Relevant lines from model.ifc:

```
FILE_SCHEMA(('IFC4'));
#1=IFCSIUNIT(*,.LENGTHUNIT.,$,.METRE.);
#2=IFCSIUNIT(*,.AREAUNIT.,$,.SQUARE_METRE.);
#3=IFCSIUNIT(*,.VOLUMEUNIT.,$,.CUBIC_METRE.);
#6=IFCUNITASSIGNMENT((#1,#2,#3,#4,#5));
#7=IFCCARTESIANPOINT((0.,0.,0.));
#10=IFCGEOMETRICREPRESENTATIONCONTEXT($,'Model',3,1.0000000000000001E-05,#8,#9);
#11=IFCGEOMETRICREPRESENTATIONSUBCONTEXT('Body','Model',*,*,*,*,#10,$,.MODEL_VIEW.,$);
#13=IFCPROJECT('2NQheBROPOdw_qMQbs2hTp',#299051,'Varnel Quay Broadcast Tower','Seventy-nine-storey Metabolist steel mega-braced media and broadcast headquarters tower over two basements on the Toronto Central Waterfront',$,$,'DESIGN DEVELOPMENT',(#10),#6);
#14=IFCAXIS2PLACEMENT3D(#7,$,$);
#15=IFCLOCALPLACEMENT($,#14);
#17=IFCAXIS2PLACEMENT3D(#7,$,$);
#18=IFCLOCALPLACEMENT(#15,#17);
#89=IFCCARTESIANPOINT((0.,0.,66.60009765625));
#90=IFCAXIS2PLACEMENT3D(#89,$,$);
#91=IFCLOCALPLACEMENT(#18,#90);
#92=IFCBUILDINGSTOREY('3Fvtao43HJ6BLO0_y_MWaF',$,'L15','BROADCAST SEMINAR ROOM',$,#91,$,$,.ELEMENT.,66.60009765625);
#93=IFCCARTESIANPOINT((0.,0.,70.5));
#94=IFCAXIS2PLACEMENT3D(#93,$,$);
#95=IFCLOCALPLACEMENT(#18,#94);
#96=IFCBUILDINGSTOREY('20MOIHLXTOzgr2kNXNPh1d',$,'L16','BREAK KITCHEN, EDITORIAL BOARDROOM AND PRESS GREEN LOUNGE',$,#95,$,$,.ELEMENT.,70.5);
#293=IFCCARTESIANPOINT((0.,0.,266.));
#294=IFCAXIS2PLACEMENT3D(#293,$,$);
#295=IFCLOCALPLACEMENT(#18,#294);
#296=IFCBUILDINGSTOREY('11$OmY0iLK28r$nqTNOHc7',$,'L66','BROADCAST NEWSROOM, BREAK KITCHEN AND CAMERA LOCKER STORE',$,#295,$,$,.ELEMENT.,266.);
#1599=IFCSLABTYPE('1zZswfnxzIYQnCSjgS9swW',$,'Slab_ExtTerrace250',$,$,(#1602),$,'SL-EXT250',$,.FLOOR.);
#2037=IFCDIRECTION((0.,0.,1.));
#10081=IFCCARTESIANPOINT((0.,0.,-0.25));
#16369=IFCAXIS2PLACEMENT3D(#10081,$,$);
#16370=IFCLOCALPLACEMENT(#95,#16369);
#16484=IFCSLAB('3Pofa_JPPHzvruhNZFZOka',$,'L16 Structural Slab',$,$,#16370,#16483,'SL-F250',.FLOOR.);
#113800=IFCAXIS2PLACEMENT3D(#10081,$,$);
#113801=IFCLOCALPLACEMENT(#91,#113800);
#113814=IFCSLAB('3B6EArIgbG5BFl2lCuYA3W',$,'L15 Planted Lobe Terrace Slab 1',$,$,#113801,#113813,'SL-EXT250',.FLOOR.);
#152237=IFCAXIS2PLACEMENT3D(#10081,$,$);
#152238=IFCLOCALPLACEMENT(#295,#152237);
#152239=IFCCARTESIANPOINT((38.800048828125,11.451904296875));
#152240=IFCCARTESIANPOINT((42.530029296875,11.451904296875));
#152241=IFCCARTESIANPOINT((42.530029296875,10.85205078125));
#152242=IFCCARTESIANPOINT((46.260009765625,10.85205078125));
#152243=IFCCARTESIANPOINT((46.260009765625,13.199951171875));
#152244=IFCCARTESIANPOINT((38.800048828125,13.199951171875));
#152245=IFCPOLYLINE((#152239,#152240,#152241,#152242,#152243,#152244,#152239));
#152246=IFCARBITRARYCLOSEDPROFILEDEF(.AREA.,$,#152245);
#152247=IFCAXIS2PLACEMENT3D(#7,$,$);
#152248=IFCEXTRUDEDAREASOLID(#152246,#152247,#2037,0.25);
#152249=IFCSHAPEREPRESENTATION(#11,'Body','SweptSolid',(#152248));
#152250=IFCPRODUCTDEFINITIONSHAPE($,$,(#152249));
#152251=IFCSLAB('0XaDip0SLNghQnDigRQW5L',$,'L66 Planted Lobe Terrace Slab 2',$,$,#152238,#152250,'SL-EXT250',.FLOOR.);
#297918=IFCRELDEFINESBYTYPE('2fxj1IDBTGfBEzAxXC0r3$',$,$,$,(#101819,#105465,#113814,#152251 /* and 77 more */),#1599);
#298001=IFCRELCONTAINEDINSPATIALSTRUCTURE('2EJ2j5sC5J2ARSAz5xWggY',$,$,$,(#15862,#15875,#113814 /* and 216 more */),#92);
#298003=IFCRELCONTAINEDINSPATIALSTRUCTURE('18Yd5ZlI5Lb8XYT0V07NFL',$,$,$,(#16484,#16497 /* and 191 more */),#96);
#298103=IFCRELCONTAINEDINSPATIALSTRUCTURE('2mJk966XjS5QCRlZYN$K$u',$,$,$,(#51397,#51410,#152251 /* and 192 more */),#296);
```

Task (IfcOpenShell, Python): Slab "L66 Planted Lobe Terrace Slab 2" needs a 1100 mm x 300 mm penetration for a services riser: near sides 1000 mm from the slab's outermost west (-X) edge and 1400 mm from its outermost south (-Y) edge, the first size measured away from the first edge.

```python
import numpy as np
import ifcopenshell
import ifcopenshell.api.feature
import ifcopenshell.api.geometry
import ifcopenshell.api.root
import ifcopenshell.geom
import ifcopenshell.util.placement
import ifcopenshell.util.representation
import ifcopenshell.util.shape
import ifcopenshell.util.unit

model = ifcopenshell.open("model.ifc")
unit_scale = ifcopenshell.util.unit.calculate_unit_scale(model)
settings = ifcopenshell.geom.settings()


def volume(element):
    """Net volume in cubic metres, openings subtracted."""
    shape = ifcopenshell.geom.create_shape(settings, element)
    return ifcopenshell.util.shape.get_volume(shape.geometry)


slab = model.by_id(152251)
before = volume(slab)

# Extent in the slab's own axes, in metres. The edges named are its -X and -Y sides.
slab_shape = ifcopenshell.geom.create_shape(settings, slab)
vertices = ifcopenshell.util.shape.get_vertices(slab_shape.geometry)
x_min, y_min, bottom = vertices.min(axis=0)
top = vertices[:, 2].max()

opening = ifcopenshell.api.root.create_entity(model, ifc_class="IfcOpeningElement", name="Services riser opening", predefined_type="OPENING")
context = ifcopenshell.util.representation.get_context(model, "Model", "Body", "MODEL_VIEW")
width, depth = 1.1, 0.3
outline = [(0.0, 0.0), (width, 0.0), (width, depth), (0.0, depth), (0.0, 0.0)]
# Overshoot both faces by 50 mm so the cut is clean.
shape = ifcopenshell.api.geometry.add_slab_representation(
    model, context=context, depth=top - bottom + 0.1, polyline=outline
)
ifcopenshell.api.geometry.assign_representation(model, product=opening, representation=shape)

matrix = ifcopenshell.util.placement.get_local_placement(slab.ObjectPlacement)
matrix[:, 3] = matrix @ np.append(np.array([x_min + 1, y_min + 1.4, bottom - 0.05]) / unit_scale, 1.0)
ifcopenshell.api.geometry.edit_object_placement(model, product=opening, matrix=matrix, is_si=False)
ifcopenshell.api.feature.add_feature(model, feature=opening, element=slab)

after = volume(slab)

print(f"slab volume {before:.3f} -> {after:.3f} m3")

model.write("model_v2.ifc")
```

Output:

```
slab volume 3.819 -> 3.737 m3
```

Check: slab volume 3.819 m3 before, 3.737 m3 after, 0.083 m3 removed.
